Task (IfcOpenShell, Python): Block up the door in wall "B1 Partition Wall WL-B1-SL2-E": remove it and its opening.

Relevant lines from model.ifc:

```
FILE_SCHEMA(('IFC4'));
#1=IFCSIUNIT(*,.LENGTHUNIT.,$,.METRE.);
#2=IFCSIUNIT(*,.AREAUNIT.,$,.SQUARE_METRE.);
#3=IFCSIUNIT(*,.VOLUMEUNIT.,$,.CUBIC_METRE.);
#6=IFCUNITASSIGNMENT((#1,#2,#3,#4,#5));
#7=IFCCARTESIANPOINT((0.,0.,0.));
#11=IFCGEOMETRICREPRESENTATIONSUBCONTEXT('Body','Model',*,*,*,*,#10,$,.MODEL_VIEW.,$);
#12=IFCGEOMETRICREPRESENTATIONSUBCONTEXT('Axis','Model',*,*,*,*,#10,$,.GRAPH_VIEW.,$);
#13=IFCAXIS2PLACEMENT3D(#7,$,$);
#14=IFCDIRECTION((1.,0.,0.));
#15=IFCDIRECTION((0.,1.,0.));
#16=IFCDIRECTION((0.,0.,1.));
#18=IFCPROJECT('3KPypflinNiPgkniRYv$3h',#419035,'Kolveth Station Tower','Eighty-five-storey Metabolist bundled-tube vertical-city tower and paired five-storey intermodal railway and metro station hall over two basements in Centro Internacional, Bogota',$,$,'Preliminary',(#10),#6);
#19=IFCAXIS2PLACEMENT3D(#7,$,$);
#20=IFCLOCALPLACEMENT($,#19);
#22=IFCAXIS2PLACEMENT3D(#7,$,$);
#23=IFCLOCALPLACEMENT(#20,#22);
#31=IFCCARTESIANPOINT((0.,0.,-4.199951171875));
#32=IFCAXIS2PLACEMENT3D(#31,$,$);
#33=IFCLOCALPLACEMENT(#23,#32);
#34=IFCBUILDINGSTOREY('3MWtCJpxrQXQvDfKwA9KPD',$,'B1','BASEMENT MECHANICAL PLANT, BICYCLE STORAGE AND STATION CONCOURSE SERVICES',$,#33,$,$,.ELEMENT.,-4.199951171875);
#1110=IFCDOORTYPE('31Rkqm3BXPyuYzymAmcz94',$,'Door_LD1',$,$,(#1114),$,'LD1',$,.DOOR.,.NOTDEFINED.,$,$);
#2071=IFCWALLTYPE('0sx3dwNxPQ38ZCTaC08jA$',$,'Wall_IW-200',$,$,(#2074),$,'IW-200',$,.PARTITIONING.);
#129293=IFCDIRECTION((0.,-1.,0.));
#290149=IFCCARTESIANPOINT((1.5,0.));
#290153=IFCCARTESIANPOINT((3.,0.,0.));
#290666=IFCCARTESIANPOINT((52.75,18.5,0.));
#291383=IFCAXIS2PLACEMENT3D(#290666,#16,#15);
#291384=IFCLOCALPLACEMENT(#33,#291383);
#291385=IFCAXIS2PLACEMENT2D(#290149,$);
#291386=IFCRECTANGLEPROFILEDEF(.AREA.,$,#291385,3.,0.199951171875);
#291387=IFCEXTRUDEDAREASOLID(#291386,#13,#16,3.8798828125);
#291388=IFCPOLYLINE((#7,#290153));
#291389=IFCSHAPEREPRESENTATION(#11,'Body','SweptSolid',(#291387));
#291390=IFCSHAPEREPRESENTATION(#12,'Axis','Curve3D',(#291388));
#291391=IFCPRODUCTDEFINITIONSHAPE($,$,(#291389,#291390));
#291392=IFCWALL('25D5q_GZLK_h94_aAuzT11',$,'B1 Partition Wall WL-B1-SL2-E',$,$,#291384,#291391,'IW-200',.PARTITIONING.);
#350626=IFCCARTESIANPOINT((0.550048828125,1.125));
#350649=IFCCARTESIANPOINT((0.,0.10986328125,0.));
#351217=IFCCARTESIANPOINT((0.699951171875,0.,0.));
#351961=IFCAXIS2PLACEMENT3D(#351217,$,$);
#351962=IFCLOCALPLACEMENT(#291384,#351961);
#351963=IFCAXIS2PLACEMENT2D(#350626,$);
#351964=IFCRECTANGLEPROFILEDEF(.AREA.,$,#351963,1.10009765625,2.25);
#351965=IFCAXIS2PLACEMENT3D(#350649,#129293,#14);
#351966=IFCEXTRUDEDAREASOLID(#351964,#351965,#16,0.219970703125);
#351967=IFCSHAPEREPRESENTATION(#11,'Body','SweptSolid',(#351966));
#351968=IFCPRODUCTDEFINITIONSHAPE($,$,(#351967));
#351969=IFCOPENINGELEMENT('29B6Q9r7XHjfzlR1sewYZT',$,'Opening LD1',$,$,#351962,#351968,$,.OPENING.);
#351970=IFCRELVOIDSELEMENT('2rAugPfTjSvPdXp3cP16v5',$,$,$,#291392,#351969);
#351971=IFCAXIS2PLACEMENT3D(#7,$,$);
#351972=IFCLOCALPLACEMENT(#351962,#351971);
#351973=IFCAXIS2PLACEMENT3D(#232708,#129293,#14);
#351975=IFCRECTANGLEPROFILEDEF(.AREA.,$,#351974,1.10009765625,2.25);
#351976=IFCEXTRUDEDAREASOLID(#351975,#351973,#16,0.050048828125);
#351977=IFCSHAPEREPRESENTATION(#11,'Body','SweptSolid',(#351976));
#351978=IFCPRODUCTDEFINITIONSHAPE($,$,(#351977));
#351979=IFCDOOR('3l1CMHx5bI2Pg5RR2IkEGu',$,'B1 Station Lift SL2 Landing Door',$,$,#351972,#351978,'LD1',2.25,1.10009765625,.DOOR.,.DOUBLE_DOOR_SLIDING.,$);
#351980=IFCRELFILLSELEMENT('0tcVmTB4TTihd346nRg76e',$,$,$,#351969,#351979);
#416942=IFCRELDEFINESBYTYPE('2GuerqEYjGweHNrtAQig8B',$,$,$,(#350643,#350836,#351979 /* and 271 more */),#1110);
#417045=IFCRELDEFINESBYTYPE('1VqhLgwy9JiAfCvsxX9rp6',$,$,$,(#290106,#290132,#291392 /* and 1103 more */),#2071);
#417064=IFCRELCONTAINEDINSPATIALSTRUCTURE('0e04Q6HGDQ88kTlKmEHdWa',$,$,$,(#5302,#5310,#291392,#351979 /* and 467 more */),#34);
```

```python
import ifcopenshell
import ifcopenshell.api.feature
import ifcopenshell.api.root
import ifcopenshell.geom
import ifcopenshell.util.shape

model = ifcopenshell.open("model.ifc")
settings = ifcopenshell.geom.settings()


def volume(element):
    """Net volume in cubic metres, openings subtracted."""
    shape = ifcopenshell.geom.create_shape(settings, element)
    return ifcopenshell.util.shape.get_volume(shape.geometry)


door = model.by_id(351979)
opening = door.FillsVoids[0].RelatingOpeningElement
wall = opening.VoidsElements[0].RelatingBuildingElement
before = volume(wall)

ifcopenshell.api.root.remove_product(model, product=door)
ifcopenshell.api.feature.remove_feature(model, feature=opening)

after = volume(wall)

print(f"wall volume {before:.3f} -> {after:.3f} m3")

model.write("model-out.ifc")
```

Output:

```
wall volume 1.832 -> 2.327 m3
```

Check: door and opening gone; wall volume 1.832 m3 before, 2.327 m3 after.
